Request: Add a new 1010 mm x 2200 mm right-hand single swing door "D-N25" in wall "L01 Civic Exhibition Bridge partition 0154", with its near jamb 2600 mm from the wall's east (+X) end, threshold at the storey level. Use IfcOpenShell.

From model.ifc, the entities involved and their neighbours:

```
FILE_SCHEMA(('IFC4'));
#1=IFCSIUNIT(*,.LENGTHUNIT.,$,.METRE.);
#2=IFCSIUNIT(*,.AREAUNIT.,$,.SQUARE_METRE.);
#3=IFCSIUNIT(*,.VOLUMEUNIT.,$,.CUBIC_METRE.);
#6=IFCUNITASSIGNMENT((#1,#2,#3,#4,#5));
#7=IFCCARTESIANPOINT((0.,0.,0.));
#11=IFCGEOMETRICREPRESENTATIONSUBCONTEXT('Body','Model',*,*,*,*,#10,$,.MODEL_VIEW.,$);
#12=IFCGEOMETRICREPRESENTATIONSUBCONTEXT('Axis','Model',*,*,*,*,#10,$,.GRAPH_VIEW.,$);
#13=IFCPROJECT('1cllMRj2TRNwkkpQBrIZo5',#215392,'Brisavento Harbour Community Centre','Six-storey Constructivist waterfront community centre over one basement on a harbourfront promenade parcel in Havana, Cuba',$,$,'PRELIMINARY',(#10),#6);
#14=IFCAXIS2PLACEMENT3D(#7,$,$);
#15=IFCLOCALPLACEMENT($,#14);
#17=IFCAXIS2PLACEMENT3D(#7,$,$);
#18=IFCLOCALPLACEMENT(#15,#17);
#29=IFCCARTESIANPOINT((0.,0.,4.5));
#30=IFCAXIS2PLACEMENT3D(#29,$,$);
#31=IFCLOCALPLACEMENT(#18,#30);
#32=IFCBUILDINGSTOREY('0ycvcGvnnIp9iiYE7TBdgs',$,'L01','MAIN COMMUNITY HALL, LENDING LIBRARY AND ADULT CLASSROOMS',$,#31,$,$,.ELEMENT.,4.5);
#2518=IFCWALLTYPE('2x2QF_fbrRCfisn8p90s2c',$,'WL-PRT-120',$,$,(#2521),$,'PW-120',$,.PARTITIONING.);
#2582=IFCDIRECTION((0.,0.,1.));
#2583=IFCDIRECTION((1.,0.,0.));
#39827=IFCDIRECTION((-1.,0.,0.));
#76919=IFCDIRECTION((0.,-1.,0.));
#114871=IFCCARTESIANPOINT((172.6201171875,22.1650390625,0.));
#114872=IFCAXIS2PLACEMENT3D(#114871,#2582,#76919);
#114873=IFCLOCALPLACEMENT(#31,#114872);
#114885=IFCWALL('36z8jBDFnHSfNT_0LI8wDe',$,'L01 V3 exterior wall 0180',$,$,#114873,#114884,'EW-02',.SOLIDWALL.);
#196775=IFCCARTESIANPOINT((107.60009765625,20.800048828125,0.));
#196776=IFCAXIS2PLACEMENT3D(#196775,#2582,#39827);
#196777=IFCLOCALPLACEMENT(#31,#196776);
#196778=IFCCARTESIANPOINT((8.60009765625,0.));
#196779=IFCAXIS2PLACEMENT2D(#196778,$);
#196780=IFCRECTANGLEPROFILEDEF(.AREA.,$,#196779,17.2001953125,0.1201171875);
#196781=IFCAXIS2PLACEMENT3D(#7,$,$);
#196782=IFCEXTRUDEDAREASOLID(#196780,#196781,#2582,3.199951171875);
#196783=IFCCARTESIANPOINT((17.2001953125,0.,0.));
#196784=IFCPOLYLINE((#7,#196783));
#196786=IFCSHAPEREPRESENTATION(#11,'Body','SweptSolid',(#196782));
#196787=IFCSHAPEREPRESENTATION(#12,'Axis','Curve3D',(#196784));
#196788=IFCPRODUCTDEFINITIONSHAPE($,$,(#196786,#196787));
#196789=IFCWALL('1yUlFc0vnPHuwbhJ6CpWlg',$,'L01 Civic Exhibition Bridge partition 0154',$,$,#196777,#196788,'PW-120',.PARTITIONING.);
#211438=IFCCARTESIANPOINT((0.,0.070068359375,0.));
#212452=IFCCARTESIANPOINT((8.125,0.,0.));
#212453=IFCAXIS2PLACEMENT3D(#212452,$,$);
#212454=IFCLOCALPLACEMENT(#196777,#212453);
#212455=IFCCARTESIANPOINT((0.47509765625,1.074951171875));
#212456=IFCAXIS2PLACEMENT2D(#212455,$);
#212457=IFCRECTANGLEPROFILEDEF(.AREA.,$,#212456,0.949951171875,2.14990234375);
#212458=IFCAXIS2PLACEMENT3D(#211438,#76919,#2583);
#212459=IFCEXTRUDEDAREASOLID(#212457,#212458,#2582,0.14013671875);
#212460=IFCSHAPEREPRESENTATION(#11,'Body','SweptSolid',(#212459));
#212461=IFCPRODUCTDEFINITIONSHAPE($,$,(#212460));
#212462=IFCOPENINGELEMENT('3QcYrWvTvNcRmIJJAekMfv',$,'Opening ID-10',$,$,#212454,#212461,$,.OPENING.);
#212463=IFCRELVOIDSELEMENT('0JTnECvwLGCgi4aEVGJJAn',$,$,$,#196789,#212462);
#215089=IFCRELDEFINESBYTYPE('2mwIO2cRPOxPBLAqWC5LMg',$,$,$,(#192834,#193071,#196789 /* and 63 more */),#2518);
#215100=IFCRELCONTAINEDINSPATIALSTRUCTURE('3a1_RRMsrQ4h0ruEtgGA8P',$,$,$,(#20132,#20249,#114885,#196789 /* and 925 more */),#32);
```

```python
import numpy as np
import ifcopenshell
import ifcopenshell.api.feature
import ifcopenshell.api.geometry
import ifcopenshell.api.root
import ifcopenshell.api.spatial
import ifcopenshell.geom
import ifcopenshell.util.element
import ifcopenshell.util.placement
import ifcopenshell.util.representation
import ifcopenshell.util.shape
import ifcopenshell.util.unit

model = ifcopenshell.open("model.ifc")
unit_scale = ifcopenshell.util.unit.calculate_unit_scale(model)
settings = ifcopenshell.geom.settings()


def volume(element):
    """Net volume in cubic metres, openings subtracted."""
    shape = ifcopenshell.geom.create_shape(settings, element)
    return ifcopenshell.util.shape.get_volume(shape.geometry)


wall = model.by_guid("1yUlFc0vnPHuwbhJ6CpWlg")
storey = ifcopenshell.util.element.get_container(wall, ifc_class="IfcBuildingStorey")
context = ifcopenshell.util.representation.get_context(model, "Model", "Body", "MODEL_VIEW")
before = volume(wall)

width, height, from_end, sill = 1.01, 2.2, 2.6, 0.0  # metres

# The wall runs along its own X axis, and the end named is its -X end.
wall_shape = ifcopenshell.geom.create_shape(settings, wall)
x, y, z = ifcopenshell.util.shape.get_vertices(wall_shape.geometry).T
start = x.min() + from_end
face, thickness = float(y.min()), float(y.max() - y.min())
wall_matrix = ifcopenshell.util.placement.get_local_placement(wall.ObjectPlacement)
level = ifcopenshell.util.placement.get_local_placement(storey.ObjectPlacement)[2, 3]


def in_wall(x, y):
    """Placement at x, y metres in the wall's axes, at sill height."""
    matrix = wall_matrix.copy()
    matrix[:, 3] = wall_matrix @ np.array([x / unit_scale, y / unit_scale, 0.0, 1.0])
    matrix[2, 3] = level + sill / unit_scale
    return matrix


# Opening: a box that overshoots both wall faces by 50 mm.
opening = ifcopenshell.api.root.create_entity(model, ifc_class="IfcOpeningElement", predefined_type="OPENING")
box = ifcopenshell.api.geometry.add_wall_representation(
    model, context=context, length=width, height=height, thickness=thickness + 0.1
)
ifcopenshell.api.geometry.assign_representation(model, product=opening, representation=box)
ifcopenshell.api.geometry.edit_object_placement(model, product=opening, matrix=in_wall(start, face - 0.05), is_si=False)
ifcopenshell.api.feature.add_feature(model, feature=opening, element=wall)

door = ifcopenshell.api.root.create_entity(model, ifc_class="IfcDoor", name="D-N25", predefined_type="DOOR")
door.OverallWidth, door.OverallHeight = width / unit_scale, height / unit_scale
door.OperationType = "SINGLE_SWING_RIGHT"
body = ifcopenshell.api.geometry.add_door_representation(
    model,
    context=context,
    overall_width=door.OverallWidth,
    overall_height=door.OverallHeight,
    operation_type="SINGLE_SWING_RIGHT",
    lining_properties={"LiningDepth": thickness / unit_scale, "ThresholdDepth": thickness / unit_scale},
)
ifcopenshell.api.geometry.assign_representation(model, product=door, representation=body)
ifcopenshell.api.spatial.assign_container(model, products=[door], relating_structure=storey)
ifcopenshell.api.feature.add_filling(model, opening=opening, element=door)

# The lining spans the wall, so the door starts at the wall face.
ifcopenshell.api.geometry.edit_object_placement(model, product=door, matrix=in_wall(start, face), is_si=False)

after = volume(wall)

print(f"wall volume {before:.3f} -> {after:.3f} m3")

model.write("model_v2.ifc")
```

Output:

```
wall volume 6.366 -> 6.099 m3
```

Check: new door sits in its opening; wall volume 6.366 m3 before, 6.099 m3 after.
